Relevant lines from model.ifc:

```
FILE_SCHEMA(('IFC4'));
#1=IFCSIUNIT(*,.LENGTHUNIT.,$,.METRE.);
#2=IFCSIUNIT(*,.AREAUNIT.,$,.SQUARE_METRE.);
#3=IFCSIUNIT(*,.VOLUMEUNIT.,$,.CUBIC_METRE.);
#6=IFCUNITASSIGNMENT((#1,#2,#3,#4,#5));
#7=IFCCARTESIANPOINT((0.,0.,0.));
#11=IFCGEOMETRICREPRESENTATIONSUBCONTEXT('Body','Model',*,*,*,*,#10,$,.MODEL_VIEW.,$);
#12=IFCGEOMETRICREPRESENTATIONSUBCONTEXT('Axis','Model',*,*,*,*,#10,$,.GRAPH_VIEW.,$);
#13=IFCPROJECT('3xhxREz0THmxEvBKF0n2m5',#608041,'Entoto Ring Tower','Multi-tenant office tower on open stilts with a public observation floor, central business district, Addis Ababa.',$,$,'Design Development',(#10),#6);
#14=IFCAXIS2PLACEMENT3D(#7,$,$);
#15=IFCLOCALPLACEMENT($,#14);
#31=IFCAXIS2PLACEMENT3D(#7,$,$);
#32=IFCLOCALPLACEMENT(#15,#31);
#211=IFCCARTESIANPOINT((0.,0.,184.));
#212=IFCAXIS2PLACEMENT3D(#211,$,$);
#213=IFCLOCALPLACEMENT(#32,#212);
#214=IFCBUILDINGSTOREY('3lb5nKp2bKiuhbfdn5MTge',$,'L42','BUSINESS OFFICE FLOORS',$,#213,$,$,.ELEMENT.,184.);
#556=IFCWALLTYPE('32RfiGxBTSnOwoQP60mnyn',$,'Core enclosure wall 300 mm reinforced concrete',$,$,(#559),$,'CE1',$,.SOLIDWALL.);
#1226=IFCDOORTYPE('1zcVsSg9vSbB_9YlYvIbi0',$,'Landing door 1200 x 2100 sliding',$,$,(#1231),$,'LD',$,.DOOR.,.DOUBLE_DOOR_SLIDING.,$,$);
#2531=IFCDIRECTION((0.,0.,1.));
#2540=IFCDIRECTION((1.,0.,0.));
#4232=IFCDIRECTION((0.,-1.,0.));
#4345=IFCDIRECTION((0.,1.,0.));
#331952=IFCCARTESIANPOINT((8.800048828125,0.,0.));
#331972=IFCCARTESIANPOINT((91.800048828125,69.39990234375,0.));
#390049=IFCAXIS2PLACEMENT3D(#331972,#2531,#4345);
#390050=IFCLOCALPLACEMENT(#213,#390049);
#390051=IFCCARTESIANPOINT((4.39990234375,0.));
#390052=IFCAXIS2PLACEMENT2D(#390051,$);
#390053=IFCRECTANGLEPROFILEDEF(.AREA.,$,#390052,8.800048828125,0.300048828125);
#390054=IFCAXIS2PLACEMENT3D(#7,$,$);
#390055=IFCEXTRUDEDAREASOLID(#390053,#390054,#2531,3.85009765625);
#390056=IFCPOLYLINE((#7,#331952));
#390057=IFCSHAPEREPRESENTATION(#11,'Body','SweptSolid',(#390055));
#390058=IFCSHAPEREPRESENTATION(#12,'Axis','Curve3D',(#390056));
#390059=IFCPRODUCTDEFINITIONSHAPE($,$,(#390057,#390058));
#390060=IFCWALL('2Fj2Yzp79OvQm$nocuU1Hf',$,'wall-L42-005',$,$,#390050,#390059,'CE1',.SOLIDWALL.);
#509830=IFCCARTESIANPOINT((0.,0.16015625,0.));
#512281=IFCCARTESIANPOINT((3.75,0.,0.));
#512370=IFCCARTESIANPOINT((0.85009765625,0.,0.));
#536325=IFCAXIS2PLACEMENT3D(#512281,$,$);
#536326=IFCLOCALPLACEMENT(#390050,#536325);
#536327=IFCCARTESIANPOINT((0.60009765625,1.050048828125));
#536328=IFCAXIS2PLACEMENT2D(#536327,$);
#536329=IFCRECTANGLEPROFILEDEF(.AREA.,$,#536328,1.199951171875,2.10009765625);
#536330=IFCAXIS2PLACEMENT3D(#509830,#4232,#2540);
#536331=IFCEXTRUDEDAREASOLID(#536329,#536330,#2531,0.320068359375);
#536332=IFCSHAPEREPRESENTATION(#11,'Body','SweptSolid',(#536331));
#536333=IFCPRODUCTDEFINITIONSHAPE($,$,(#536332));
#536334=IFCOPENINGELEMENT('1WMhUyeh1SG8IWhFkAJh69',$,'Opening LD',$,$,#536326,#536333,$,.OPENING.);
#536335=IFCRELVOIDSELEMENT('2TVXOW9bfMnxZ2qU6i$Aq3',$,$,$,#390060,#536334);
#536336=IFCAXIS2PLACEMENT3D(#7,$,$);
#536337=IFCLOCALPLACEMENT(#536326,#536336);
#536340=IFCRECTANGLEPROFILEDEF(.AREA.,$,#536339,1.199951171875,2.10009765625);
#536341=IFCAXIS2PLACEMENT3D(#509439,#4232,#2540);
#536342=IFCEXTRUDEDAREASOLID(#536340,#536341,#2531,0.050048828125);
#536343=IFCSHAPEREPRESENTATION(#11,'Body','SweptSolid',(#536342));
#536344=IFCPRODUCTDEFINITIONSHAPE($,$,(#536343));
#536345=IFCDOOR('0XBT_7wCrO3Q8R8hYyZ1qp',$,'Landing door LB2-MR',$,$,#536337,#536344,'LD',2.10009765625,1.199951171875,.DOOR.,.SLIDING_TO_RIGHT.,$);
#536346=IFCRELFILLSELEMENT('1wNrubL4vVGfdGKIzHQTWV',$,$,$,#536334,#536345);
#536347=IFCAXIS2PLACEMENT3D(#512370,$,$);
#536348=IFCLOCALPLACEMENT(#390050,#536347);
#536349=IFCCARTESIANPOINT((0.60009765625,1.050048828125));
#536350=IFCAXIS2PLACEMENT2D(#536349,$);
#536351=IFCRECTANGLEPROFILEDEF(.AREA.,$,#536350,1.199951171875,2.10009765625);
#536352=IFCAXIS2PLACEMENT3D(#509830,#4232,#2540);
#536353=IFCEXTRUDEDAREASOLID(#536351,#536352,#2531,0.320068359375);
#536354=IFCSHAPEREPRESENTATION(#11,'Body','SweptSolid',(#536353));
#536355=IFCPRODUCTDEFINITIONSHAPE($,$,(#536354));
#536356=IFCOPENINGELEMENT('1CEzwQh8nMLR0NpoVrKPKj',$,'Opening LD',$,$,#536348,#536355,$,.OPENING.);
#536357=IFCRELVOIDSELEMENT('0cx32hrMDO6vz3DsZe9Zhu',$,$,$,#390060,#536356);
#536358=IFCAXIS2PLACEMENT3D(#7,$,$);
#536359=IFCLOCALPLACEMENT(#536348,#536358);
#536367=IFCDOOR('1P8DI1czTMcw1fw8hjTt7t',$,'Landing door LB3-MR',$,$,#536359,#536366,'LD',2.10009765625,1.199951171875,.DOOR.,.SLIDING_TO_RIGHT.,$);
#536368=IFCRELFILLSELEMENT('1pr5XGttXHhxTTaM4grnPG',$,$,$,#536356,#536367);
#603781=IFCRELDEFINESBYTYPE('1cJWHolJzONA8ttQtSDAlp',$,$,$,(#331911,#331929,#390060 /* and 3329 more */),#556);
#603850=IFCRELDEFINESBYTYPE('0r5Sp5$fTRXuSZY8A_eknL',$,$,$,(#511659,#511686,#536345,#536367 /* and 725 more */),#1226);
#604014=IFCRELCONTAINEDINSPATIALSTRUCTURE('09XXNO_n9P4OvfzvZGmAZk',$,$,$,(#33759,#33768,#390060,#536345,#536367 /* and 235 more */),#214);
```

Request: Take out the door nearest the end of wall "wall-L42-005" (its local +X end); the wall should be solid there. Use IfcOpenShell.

```python
import ifcopenshell
import ifcopenshell.api.feature
import ifcopenshell.api.root
import ifcopenshell.geom
import ifcopenshell.util.shape

model = ifcopenshell.open("model.ifc")
settings = ifcopenshell.geom.settings()


def volume(element):
    """Net volume in cubic metres, openings subtracted."""
    shape = ifcopenshell.geom.create_shape(settings, element)
    return ifcopenshell.util.shape.get_volume(shape.geometry)


door = model.by_guid("0XBT_7wCrO3Q8R8hYyZ1qp")
opening = door.FillsVoids[0].RelatingOpeningElement
wall = opening.VoidsElements[0].RelatingBuildingElement
before = volume(wall)

ifcopenshell.api.root.remove_product(model, product=door)
ifcopenshell.api.feature.remove_feature(model, feature=opening)

after = volume(wall)

print(f"wall volume {before:.3f} -> {after:.3f} m3")

model.write("model_edited.ifc")
```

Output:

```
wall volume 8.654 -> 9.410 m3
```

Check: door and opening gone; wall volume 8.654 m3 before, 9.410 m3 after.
